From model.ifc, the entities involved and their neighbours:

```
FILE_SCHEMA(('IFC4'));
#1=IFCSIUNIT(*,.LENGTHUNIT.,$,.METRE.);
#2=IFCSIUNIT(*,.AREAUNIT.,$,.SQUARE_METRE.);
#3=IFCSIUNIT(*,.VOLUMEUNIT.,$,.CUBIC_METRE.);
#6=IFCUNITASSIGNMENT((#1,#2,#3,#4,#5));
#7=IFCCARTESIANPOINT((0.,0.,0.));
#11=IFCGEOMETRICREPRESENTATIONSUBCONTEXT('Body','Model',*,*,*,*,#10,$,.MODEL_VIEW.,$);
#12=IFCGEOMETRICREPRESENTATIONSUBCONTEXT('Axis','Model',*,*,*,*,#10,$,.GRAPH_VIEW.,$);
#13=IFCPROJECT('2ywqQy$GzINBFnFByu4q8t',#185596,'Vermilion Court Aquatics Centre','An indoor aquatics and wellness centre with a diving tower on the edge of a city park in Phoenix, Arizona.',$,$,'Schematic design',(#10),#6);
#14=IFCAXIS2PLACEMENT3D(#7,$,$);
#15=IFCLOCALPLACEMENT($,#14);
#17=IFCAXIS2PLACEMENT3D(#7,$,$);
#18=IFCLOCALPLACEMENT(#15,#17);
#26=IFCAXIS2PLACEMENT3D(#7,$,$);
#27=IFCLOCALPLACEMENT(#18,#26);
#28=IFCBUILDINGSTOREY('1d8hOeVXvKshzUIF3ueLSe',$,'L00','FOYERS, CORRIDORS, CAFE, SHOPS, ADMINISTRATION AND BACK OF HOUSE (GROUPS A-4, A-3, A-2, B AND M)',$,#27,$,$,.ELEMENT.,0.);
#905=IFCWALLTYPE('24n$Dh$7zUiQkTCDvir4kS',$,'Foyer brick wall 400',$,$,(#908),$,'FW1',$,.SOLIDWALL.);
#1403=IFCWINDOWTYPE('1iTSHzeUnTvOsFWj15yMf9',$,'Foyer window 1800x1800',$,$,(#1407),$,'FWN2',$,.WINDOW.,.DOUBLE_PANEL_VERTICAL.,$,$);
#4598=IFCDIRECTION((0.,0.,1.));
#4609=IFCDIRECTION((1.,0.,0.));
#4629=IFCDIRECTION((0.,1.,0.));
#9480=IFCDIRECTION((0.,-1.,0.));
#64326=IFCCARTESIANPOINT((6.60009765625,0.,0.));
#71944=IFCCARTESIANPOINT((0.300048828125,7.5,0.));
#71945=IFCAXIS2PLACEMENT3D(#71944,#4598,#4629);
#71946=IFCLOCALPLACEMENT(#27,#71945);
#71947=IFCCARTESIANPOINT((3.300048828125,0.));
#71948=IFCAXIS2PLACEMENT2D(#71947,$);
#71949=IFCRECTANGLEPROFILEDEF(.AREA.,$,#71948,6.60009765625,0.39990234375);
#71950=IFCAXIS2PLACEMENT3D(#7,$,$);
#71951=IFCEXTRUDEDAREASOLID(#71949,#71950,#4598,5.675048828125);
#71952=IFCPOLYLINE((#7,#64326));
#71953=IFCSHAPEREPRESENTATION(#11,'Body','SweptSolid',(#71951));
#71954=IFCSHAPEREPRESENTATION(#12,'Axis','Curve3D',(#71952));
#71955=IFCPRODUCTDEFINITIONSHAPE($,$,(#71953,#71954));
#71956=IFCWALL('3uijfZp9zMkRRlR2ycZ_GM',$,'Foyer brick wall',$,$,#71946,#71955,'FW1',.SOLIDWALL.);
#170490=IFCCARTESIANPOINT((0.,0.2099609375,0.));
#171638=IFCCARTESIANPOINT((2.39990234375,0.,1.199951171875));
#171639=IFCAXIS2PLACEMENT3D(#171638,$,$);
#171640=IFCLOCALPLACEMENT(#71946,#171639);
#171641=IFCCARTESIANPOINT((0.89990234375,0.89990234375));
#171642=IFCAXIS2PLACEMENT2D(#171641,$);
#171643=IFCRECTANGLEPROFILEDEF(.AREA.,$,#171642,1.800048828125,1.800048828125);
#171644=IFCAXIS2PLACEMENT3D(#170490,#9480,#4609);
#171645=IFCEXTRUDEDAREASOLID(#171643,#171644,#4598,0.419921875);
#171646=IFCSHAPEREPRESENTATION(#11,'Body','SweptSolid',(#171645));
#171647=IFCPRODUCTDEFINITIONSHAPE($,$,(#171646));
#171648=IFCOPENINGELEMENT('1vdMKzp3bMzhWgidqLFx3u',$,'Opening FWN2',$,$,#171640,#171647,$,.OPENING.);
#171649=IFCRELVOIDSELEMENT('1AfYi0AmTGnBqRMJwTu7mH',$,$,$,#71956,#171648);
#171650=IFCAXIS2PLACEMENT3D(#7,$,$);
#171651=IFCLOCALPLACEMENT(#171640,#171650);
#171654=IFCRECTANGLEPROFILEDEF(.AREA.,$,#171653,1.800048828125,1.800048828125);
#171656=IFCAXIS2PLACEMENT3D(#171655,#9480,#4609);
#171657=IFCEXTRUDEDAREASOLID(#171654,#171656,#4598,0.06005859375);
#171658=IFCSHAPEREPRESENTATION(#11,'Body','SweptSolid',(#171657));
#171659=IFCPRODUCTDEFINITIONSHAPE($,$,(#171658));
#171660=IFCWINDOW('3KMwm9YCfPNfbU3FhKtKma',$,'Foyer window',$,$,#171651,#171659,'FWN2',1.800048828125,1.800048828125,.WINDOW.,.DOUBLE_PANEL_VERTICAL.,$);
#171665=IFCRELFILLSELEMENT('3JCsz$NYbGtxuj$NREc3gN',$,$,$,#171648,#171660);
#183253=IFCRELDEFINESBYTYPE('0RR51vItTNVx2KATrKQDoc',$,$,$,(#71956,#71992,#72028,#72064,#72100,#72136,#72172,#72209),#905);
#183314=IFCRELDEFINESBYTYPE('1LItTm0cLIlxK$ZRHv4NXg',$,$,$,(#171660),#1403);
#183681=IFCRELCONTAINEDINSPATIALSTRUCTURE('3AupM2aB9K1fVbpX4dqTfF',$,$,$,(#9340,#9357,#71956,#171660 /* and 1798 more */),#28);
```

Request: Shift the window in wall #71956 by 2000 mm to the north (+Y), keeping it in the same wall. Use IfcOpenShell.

```python
import ifcopenshell
import ifcopenshell.api.geometry
import ifcopenshell.util.placement
import ifcopenshell.util.unit

model = ifcopenshell.open("model.ifc")
unit_scale = ifcopenshell.util.unit.calculate_unit_scale(model)

window = model.by_guid("3KMwm9YCfPNfbU3FhKtKma")
opening = window.FillsVoids[0].RelatingOpeningElement
wall = opening.VoidsElements[0].RelatingBuildingElement

wall_matrix = ifcopenshell.util.placement.get_local_placement(wall.ObjectPlacement)
shift = wall_matrix[:3, 0] * 2 / unit_scale
before = ifcopenshell.util.placement.get_local_placement(window.ObjectPlacement)[:3, 3].copy()

# The window is placed relative to its opening, so it follows when the opening moves.
matrix = ifcopenshell.util.placement.get_local_placement(opening.ObjectPlacement)
matrix[:3, 3] += shift
ifcopenshell.api.geometry.edit_object_placement(
    model, product=opening, matrix=matrix, is_si=False, should_transform_children=True
)

after = ifcopenshell.util.placement.get_local_placement(window.ObjectPlacement)[:3, 3]
print("window moved by", (after - before).round(3) + 0.0)

model.write("model_rev.ifc")
```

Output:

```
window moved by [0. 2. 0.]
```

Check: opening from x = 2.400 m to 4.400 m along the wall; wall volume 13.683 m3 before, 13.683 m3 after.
